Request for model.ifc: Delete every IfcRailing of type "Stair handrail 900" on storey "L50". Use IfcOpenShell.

First a look at what the model holds.

```python
import ifcopenshell
import ifcopenshell.util.element

model = ifcopenshell.open("model.ifc")
print(model.schema)
storey = next(s for s in model.by_type("IfcBuildingStorey") if s.Name == "L50")
railings = [e for e in ifcopenshell.util.element.get_decomposition(storey) if e.is_a("IfcRailing")]
seen = {}
for e in railings:
    element_type = ifcopenshell.util.element.get_type(e)
    name = element_type.Name if element_type not in (None, e) else None
    seen[name] = seen.get(name, 0) + 1
for name, count in sorted(seen.items(), key=str):
    print(count, "x", name)
```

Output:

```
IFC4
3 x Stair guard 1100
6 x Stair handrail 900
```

```python
import ifcopenshell
import ifcopenshell.api.root
import ifcopenshell.util.element

model = ifcopenshell.open("model.ifc")

storey = next(s for s in model.by_type("IfcBuildingStorey") if s.Name == "L50")
railings = [e for e in ifcopenshell.util.element.get_decomposition(storey) if e.is_a("IfcRailing")]
targets = [e for e in railings if (t := ifcopenshell.util.element.get_type(e)) not in (None, e) and t.Name == "Stair handrail 900"]

for e in targets:
    ifcopenshell.api.root.remove_product(model, product=e)
print(len(targets), "removed")

model.write("model_rev.ifc")
```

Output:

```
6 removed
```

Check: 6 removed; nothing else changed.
